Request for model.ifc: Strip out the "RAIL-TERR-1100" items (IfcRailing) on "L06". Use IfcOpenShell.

First a look at what the model holds.

```python
import ifcopenshell
import ifcopenshell.util.element

model = ifcopenshell.open("model.ifc")
print(model.schema)
storey = next(s for s in model.by_type("IfcBuildingStorey") if s.Name == "L06")
railings = [e for e in ifcopenshell.util.element.get_decomposition(storey) if e.is_a("IfcRailing")]
seen = {}
for e in railings:
    element_type = ifcopenshell.util.element.get_type(e)
    name = element_type.Name if element_type not in (None, e) else None
    seen[name] = seen.get(name, 0) + 1
for name, count in sorted(seen.items(), key=str):
    print(count, "x", name)
```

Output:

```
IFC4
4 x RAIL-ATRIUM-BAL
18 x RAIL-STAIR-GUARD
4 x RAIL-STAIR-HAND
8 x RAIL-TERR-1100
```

```python
import ifcopenshell
import ifcopenshell.api.root
import ifcopenshell.util.element

model = ifcopenshell.open("model.ifc")

storey = next(s for s in model.by_type("IfcBuildingStorey") if s.Name == "L06")
railings = [e for e in ifcopenshell.util.element.get_decomposition(storey) if e.is_a("IfcRailing")]
targets = [e for e in railings if (t := ifcopenshell.util.element.get_type(e)) not in (None, e) and t.Name == "RAIL-TERR-1100"]

for e in targets:
    ifcopenshell.api.root.remove_product(model, product=e)
print(len(targets), "removed")

model.write("model_updated.ifc")
```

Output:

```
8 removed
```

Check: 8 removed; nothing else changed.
